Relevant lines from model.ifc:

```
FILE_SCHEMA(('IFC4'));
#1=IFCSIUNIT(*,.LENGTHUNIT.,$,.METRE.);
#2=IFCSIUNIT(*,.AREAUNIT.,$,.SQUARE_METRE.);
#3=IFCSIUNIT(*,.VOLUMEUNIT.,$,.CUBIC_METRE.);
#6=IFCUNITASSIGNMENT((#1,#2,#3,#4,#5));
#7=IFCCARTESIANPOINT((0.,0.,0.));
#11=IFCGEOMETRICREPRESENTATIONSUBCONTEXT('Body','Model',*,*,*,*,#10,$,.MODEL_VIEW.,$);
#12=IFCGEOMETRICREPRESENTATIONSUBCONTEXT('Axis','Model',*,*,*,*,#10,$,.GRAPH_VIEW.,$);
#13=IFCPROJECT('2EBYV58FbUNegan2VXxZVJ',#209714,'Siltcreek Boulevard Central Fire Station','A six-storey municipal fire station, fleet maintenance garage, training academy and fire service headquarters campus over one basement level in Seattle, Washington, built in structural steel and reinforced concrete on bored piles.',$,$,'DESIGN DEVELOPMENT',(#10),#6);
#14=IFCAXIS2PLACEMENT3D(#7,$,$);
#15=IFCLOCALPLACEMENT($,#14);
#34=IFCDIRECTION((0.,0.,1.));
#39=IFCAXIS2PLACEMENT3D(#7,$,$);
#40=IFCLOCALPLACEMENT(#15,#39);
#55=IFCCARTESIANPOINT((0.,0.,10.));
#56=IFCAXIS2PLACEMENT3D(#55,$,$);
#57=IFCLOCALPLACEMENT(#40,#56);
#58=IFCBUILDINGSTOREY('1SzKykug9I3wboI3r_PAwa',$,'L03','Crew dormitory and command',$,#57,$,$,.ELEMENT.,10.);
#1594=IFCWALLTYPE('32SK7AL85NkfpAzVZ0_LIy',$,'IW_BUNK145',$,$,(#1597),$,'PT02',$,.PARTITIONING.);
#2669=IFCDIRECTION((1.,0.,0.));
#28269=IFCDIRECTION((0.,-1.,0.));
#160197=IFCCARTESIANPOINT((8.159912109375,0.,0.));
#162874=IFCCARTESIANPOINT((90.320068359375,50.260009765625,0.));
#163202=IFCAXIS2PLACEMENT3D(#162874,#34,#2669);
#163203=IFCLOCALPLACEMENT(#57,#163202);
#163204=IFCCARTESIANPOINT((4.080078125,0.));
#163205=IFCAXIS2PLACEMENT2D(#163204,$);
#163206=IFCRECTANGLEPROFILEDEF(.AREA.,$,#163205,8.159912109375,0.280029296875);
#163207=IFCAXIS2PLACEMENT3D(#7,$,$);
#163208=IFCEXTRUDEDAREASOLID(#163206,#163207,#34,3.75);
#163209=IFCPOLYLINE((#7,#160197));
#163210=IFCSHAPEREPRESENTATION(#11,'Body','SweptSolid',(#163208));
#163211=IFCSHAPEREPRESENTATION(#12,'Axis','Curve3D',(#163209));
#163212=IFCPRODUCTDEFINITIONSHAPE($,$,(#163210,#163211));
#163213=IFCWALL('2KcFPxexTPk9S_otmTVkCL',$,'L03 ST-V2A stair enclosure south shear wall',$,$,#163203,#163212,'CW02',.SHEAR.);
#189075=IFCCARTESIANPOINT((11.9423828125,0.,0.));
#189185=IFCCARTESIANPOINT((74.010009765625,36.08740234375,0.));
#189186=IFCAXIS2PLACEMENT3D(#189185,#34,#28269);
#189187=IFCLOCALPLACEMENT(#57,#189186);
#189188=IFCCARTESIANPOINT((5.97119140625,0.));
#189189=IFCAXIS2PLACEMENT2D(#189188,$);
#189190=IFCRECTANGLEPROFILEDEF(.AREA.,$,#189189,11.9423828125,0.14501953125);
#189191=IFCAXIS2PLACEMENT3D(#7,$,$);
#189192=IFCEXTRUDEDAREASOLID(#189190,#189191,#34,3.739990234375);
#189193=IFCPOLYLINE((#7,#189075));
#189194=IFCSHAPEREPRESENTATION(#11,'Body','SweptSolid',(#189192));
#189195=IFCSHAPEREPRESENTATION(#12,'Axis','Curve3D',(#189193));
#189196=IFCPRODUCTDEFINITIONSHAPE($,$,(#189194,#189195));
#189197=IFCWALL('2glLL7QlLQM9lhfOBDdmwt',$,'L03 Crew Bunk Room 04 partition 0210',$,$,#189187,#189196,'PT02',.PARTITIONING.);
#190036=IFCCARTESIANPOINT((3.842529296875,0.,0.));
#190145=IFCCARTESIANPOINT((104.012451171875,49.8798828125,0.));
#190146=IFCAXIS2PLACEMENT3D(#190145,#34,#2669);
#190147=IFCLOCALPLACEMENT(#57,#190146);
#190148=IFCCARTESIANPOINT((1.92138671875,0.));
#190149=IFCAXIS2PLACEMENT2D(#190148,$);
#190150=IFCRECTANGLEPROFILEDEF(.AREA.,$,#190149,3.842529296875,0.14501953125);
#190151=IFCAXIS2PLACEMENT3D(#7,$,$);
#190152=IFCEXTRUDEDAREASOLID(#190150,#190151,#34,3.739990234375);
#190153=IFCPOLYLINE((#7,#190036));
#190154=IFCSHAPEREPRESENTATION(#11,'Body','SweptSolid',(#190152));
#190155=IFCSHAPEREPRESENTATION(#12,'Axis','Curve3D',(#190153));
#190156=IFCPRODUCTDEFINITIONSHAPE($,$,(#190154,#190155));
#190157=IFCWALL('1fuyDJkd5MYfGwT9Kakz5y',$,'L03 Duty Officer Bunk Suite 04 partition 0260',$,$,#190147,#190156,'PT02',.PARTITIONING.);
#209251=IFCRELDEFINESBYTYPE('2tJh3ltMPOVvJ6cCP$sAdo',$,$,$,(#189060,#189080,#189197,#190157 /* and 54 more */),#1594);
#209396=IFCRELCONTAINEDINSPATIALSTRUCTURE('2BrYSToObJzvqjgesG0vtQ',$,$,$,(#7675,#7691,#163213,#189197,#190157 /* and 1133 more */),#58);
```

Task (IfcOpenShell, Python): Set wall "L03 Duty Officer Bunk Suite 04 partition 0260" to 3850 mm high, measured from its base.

```python
import ifcopenshell
import ifcopenshell.geom
import ifcopenshell.util.representation
import ifcopenshell.util.shape

model = ifcopenshell.open("model.ifc")
settings = ifcopenshell.geom.settings()


def volume(element):
    """Net volume in cubic metres, openings subtracted."""
    shape = ifcopenshell.geom.create_shape(settings, element)
    return ifcopenshell.util.shape.get_volume(shape.geometry)


wall = model.by_guid("1fuyDJkd5MYfGwT9Kakz5y")
before = volume(wall)

body = ifcopenshell.util.representation.get_representation(wall, "Model", "Body")
solid = body.Items[0]
old_height = solid.Depth
solid.Depth = 3.85
after = volume(wall)

print(f"height {old_height:g} -> {solid.Depth:g}, volume {before:.3f} -> {after:.3f} m3")

model.write("model_rev.ifc")
```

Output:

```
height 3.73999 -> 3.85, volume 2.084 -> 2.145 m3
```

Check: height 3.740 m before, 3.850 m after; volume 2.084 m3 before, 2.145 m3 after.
